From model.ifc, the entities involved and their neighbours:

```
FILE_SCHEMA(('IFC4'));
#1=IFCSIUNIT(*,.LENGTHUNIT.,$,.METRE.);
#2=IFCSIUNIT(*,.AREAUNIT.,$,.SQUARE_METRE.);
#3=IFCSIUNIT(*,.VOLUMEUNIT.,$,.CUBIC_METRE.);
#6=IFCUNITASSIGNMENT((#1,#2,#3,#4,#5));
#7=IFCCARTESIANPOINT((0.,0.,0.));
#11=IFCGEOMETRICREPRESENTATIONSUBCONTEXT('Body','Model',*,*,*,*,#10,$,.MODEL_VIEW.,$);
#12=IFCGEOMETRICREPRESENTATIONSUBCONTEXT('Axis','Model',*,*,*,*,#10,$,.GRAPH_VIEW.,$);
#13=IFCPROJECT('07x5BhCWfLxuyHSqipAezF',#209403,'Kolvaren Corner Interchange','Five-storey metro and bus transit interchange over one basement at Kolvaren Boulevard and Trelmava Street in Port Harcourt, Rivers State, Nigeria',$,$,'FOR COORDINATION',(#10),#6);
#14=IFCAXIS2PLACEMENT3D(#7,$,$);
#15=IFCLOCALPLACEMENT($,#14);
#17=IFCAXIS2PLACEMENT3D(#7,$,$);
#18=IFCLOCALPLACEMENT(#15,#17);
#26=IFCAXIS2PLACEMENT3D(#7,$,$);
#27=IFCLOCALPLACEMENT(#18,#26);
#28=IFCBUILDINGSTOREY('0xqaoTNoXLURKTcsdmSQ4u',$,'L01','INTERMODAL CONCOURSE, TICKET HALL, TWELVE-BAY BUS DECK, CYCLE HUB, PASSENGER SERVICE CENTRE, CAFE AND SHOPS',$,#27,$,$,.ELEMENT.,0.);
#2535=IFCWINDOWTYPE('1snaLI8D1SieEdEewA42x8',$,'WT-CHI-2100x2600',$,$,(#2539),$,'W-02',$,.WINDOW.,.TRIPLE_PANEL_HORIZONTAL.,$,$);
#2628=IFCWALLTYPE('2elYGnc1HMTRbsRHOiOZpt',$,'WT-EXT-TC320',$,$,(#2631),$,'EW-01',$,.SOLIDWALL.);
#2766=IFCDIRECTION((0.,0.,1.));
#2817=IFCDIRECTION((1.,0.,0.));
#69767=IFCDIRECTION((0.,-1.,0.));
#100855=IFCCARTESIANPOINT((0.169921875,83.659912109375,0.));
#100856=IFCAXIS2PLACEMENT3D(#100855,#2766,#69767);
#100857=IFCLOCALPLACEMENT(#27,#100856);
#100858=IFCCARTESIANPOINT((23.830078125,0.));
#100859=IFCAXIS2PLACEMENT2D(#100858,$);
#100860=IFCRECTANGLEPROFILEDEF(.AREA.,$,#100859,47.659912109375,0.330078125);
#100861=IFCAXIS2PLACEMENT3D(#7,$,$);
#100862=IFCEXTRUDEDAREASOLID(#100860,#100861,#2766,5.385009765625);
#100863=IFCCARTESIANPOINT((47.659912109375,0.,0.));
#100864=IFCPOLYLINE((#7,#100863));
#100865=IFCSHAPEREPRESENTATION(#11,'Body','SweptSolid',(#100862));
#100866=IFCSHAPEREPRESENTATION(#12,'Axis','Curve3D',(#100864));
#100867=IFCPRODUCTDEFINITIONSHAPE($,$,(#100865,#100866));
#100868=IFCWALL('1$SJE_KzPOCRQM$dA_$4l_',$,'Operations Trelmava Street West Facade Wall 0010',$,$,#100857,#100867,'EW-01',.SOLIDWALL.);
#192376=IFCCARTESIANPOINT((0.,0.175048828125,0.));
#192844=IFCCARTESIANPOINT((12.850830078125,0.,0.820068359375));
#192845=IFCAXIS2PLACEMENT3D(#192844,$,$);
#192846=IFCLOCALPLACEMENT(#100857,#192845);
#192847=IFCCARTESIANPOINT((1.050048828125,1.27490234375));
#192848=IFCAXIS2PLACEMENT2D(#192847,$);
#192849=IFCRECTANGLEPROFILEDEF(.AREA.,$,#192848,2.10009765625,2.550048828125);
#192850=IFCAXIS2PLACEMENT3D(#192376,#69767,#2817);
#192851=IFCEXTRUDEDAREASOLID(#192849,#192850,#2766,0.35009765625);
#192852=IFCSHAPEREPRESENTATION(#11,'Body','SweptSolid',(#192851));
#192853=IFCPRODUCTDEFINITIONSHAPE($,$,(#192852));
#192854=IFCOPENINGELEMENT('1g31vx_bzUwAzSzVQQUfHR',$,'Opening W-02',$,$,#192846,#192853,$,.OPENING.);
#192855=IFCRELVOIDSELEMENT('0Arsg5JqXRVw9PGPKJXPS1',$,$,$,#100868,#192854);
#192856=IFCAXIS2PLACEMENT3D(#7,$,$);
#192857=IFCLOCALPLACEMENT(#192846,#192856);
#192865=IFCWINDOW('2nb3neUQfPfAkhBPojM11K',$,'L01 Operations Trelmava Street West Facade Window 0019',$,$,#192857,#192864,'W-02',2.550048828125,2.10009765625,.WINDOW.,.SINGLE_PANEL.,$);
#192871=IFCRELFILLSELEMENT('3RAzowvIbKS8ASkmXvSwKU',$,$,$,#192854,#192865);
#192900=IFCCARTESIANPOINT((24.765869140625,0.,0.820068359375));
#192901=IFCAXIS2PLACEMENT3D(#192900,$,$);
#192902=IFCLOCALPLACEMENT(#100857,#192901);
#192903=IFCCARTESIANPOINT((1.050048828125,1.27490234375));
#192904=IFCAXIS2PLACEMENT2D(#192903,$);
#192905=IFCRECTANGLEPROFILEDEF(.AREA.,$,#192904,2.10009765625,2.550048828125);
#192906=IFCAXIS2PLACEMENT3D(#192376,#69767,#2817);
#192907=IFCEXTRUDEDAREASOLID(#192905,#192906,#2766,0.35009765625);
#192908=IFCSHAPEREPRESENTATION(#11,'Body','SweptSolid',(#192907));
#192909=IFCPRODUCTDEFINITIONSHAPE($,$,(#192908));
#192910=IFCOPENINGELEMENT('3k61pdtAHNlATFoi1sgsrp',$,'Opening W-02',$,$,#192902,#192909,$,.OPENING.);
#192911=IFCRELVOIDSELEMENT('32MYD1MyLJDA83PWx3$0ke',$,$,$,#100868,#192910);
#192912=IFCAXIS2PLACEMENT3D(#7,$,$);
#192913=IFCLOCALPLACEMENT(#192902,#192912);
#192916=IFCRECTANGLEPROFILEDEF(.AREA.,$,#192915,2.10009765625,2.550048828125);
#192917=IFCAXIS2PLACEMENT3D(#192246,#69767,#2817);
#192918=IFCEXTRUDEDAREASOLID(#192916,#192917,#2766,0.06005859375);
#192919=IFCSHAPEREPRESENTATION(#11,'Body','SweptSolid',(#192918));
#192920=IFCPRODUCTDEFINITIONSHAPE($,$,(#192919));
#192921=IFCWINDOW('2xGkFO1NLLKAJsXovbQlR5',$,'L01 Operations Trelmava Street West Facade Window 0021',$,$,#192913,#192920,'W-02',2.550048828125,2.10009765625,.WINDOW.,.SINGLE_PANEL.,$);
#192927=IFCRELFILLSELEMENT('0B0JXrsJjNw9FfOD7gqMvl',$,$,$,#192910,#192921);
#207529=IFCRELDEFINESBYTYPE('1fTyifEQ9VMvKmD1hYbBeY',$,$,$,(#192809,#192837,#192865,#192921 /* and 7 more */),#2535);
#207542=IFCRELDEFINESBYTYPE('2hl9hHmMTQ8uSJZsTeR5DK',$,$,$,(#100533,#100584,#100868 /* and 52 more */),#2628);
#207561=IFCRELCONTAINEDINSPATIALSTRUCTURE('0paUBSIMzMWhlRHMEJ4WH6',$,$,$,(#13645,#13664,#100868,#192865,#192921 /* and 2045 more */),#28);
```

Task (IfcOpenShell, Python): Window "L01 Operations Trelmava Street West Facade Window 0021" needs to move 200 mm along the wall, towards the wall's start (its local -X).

```python
import ifcopenshell
import ifcopenshell.api.geometry
import ifcopenshell.util.placement
import ifcopenshell.util.unit

model = ifcopenshell.open("model.ifc")
unit_scale = ifcopenshell.util.unit.calculate_unit_scale(model)

window = model.by_id(192921)
opening = window.FillsVoids[0].RelatingOpeningElement
wall = opening.VoidsElements[0].RelatingBuildingElement

wall_matrix = ifcopenshell.util.placement.get_local_placement(wall.ObjectPlacement)
shift = wall_matrix[:3, 0] * -0.2 / unit_scale
before = ifcopenshell.util.placement.get_local_placement(window.ObjectPlacement)[:3, 3].copy()

# The window is placed relative to its opening, so it follows when the opening moves.
matrix = ifcopenshell.util.placement.get_local_placement(opening.ObjectPlacement)
matrix[:3, 3] += shift
ifcopenshell.api.geometry.edit_object_placement(
    model, product=opening, matrix=matrix, is_si=False, should_transform_children=True
)

after = ifcopenshell.util.placement.get_local_placement(window.ObjectPlacement)[:3, 3]
print("window moved by", (after - before).round(3) + 0.0)

model.write("model_v2.ifc")
```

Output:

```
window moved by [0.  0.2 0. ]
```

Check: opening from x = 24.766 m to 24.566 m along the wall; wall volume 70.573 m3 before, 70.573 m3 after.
